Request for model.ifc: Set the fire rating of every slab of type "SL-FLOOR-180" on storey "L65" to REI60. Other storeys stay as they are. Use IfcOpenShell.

First a look at what the model holds.

```python
import ifcopenshell
import ifcopenshell.util.element

model = ifcopenshell.open("model.ifc")
print(model.schema)
storey = next(s for s in model.by_type("IfcBuildingStorey") if s.Name == "L65")
slabs = [e for e in ifcopenshell.util.element.get_decomposition(storey) if e.is_a("IfcSlab")]
seen = {}
for e in slabs:
    element_type = ifcopenshell.util.element.get_type(e)
    key = (element_type.Name if element_type != e and element_type else None, ifcopenshell.util.element.get_pset(e, "Pset_SlabCommon", "FireRating"))
    seen[key] = seen.get(key, 0) + 1
for (name, value), count in sorted(seen.items(), key=str):
    print(count, "x", name, "|", value)
```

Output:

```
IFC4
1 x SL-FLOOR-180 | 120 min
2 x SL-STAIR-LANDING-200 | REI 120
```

```python
import ifcopenshell
import ifcopenshell.api.pset
import ifcopenshell.util.element

model = ifcopenshell.open("model.ifc")

storey = next(s for s in model.by_type("IfcBuildingStorey") if s.Name == "L65")
slabs = [e for e in ifcopenshell.util.element.get_decomposition(storey) if e.is_a("IfcSlab")]

count = 0
for e in slabs:
    element_type = ifcopenshell.util.element.get_type(e)
    if element_type in (None, e) or element_type.Name != "SL-FLOOR-180":
        continue
    # add_pset returns the element's existing set when there is one.
    pset = ifcopenshell.api.pset.add_pset(model, product=e, name="Pset_SlabCommon")
    ifcopenshell.api.pset.edit_pset(model, pset=pset, properties={"FireRating": "REI60"})
    count += 1

print(count, "slabs updated")

model.write("model_updated.ifc")
```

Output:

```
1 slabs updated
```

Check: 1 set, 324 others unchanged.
